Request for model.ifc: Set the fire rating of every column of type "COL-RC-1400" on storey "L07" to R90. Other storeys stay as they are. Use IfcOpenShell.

First a look at what the model holds.

```python
import ifcopenshell
import ifcopenshell.util.element

model = ifcopenshell.open("model.ifc")
print(model.schema)
storey = next(s for s in model.by_type("IfcBuildingStorey") if s.Name == "L07")
columns = [e for e in ifcopenshell.util.element.get_decomposition(storey) if e.is_a("IfcColumn")]
seen = {}
for e in columns:
    element_type = ifcopenshell.util.element.get_type(e)
    key = (element_type.Name if element_type != e and element_type else None, ifcopenshell.util.element.get_pset(e, "Pset_ColumnCommon", "FireRating"))
    seen[key] = seen.get(key, 0) + 1
for (name, value), count in sorted(seen.items(), key=str):
    print(count, "x", name, "|", value)
```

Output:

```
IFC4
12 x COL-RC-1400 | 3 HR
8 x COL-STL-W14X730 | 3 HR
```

```python
import ifcopenshell
import ifcopenshell.api.pset
import ifcopenshell.util.element

model = ifcopenshell.open("model.ifc")

storey = next(s for s in model.by_type("IfcBuildingStorey") if s.Name == "L07")
columns = [e for e in ifcopenshell.util.element.get_decomposition(storey) if e.is_a("IfcColumn")]

count = 0
for e in columns:
    element_type = ifcopenshell.util.element.get_type(e)
    if element_type in (None, e) or element_type.Name != "COL-RC-1400":
        continue
    # add_pset returns the element's existing set when there is one.
    pset = ifcopenshell.api.pset.add_pset(model, product=e, name="Pset_ColumnCommon")
    ifcopenshell.api.pset.edit_pset(model, pset=pset, properties={"FireRating": "R90"})
    count += 1

print(count, "columns updated")

model.write("model_updated.ifc")
```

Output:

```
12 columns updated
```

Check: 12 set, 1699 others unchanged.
